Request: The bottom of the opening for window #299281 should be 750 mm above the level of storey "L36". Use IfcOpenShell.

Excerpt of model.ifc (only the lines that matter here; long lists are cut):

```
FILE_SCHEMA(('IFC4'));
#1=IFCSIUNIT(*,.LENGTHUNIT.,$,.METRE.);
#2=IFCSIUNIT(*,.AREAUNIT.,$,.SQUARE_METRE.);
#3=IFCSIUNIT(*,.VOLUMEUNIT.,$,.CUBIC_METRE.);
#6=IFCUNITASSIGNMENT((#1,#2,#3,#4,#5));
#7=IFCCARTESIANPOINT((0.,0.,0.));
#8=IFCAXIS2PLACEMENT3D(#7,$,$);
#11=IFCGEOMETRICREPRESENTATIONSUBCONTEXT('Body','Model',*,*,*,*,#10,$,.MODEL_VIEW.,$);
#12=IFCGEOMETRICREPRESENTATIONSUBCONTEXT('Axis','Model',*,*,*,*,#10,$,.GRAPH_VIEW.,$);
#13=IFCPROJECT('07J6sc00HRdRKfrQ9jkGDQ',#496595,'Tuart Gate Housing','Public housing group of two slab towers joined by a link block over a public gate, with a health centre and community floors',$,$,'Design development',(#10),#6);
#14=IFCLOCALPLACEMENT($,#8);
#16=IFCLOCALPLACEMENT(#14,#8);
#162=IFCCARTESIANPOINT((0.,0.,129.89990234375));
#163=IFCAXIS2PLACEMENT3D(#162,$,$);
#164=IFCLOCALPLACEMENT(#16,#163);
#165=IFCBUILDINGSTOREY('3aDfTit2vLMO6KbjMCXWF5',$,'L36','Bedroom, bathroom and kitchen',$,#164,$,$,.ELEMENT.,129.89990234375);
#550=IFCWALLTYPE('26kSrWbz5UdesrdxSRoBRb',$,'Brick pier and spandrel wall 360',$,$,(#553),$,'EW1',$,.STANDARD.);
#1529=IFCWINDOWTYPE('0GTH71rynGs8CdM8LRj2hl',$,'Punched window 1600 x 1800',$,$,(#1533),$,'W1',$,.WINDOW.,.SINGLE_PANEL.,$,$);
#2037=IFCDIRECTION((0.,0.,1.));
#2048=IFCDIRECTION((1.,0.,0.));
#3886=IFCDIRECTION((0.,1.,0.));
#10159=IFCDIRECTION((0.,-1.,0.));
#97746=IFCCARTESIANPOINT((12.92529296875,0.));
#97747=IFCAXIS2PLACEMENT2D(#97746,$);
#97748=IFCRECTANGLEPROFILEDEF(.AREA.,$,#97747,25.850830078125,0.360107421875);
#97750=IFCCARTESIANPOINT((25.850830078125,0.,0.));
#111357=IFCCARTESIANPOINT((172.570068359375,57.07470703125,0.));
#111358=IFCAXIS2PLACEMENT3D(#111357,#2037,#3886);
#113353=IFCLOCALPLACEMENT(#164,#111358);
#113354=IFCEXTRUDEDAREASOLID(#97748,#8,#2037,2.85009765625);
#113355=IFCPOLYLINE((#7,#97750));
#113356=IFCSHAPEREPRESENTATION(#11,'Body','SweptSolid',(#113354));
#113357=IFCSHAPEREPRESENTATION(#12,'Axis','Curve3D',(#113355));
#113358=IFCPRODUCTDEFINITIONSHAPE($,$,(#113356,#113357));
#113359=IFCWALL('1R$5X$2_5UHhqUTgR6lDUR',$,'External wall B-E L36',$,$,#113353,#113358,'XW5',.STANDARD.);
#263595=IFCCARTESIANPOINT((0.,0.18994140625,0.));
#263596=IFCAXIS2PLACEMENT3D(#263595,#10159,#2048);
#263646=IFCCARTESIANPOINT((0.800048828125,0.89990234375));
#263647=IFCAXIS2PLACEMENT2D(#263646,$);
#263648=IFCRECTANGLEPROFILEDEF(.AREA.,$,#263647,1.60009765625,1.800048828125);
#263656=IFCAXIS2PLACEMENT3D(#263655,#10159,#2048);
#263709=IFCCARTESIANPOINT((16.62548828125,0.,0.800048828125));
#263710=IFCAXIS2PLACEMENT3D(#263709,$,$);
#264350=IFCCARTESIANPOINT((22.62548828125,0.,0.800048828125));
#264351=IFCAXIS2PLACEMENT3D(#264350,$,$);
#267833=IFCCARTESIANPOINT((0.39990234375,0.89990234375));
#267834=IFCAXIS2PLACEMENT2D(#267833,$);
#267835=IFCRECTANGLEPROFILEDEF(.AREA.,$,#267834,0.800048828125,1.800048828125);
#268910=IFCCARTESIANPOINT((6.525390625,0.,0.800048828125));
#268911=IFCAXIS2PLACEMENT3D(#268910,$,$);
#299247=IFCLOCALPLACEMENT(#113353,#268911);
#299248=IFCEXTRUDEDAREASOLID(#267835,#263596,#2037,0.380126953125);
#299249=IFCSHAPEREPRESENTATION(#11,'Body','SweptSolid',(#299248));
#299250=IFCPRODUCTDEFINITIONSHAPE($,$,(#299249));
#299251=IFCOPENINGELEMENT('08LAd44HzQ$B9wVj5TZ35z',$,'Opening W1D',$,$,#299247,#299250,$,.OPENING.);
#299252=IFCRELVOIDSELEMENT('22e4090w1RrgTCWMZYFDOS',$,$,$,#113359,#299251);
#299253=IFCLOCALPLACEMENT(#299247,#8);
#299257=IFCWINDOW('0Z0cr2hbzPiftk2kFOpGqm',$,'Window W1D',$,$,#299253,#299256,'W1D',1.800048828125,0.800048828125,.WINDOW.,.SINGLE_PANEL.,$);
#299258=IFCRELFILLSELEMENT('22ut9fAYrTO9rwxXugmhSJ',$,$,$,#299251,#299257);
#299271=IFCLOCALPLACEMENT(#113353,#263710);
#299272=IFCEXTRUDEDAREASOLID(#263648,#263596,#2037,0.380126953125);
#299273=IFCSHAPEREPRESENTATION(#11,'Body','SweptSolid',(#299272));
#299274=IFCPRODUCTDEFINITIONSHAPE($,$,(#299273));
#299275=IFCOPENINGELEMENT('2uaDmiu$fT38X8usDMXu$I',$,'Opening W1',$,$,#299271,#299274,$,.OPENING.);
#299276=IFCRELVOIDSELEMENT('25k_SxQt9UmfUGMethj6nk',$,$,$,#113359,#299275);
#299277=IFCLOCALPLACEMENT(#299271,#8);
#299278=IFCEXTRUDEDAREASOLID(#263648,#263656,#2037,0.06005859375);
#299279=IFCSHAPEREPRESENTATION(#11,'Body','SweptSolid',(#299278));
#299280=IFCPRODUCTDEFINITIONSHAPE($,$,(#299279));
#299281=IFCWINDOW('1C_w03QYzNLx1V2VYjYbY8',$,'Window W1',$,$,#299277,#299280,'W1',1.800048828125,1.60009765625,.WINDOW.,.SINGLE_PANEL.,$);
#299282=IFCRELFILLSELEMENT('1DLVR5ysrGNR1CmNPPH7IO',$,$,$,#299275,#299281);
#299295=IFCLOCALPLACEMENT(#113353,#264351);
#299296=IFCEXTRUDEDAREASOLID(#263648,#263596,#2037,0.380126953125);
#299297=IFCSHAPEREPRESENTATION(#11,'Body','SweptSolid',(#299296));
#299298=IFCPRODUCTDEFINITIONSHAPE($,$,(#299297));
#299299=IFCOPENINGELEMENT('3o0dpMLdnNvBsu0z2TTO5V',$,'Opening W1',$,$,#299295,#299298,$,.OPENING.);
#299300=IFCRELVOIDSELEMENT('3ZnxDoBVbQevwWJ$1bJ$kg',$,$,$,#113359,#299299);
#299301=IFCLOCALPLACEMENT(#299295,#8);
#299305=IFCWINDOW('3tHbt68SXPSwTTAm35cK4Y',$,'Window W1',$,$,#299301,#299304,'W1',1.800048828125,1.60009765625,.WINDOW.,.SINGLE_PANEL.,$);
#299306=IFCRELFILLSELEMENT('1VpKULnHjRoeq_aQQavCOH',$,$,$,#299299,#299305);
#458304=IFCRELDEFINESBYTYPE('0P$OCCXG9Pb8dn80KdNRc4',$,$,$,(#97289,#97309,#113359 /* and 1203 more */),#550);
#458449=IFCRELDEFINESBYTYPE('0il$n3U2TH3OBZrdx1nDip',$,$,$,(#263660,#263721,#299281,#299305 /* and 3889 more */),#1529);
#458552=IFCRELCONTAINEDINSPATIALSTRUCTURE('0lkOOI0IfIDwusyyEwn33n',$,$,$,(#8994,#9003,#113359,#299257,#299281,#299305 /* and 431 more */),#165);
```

```python
import numpy as np
import ifcopenshell
import ifcopenshell.api.geometry
import ifcopenshell.geom
import ifcopenshell.util.element
import ifcopenshell.util.placement
import ifcopenshell.util.shape
import ifcopenshell.util.unit

model = ifcopenshell.open("model.ifc")
unit_scale = ifcopenshell.util.unit.calculate_unit_scale(model)

window = model.by_guid("1C_w03QYzNLx1V2VYjYbY8")
opening = window.FillsVoids[0].RelatingOpeningElement
storey = ifcopenshell.util.element.get_container(window, ifc_class="IfcBuildingStorey")
level = ifcopenshell.util.placement.get_local_placement(storey.ObjectPlacement)[2, 3]

# The opening's origin need not be at the sill, so measure its lowest point.
shape = ifcopenshell.geom.create_shape(ifcopenshell.geom.settings(), opening)
bottom = ifcopenshell.util.shape.get_shape_bottom_elevation(shape, shape.geometry) / unit_scale
dz = level + 0.75 / unit_scale - bottom

shift = np.array([0.0, 0.0, dz])
# The window is placed relative to its opening, so it follows when the opening moves.
matrix = ifcopenshell.util.placement.get_local_placement(opening.ObjectPlacement)
matrix[:3, 3] += shift
ifcopenshell.api.geometry.edit_object_placement(
    model, product=opening, matrix=matrix, is_si=False, should_transform_children=True
)

print(f"moved by {dz * unit_scale:+.3f} m")

model.write("model_rev.ifc")
```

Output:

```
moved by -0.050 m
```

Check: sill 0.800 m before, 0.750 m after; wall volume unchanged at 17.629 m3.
